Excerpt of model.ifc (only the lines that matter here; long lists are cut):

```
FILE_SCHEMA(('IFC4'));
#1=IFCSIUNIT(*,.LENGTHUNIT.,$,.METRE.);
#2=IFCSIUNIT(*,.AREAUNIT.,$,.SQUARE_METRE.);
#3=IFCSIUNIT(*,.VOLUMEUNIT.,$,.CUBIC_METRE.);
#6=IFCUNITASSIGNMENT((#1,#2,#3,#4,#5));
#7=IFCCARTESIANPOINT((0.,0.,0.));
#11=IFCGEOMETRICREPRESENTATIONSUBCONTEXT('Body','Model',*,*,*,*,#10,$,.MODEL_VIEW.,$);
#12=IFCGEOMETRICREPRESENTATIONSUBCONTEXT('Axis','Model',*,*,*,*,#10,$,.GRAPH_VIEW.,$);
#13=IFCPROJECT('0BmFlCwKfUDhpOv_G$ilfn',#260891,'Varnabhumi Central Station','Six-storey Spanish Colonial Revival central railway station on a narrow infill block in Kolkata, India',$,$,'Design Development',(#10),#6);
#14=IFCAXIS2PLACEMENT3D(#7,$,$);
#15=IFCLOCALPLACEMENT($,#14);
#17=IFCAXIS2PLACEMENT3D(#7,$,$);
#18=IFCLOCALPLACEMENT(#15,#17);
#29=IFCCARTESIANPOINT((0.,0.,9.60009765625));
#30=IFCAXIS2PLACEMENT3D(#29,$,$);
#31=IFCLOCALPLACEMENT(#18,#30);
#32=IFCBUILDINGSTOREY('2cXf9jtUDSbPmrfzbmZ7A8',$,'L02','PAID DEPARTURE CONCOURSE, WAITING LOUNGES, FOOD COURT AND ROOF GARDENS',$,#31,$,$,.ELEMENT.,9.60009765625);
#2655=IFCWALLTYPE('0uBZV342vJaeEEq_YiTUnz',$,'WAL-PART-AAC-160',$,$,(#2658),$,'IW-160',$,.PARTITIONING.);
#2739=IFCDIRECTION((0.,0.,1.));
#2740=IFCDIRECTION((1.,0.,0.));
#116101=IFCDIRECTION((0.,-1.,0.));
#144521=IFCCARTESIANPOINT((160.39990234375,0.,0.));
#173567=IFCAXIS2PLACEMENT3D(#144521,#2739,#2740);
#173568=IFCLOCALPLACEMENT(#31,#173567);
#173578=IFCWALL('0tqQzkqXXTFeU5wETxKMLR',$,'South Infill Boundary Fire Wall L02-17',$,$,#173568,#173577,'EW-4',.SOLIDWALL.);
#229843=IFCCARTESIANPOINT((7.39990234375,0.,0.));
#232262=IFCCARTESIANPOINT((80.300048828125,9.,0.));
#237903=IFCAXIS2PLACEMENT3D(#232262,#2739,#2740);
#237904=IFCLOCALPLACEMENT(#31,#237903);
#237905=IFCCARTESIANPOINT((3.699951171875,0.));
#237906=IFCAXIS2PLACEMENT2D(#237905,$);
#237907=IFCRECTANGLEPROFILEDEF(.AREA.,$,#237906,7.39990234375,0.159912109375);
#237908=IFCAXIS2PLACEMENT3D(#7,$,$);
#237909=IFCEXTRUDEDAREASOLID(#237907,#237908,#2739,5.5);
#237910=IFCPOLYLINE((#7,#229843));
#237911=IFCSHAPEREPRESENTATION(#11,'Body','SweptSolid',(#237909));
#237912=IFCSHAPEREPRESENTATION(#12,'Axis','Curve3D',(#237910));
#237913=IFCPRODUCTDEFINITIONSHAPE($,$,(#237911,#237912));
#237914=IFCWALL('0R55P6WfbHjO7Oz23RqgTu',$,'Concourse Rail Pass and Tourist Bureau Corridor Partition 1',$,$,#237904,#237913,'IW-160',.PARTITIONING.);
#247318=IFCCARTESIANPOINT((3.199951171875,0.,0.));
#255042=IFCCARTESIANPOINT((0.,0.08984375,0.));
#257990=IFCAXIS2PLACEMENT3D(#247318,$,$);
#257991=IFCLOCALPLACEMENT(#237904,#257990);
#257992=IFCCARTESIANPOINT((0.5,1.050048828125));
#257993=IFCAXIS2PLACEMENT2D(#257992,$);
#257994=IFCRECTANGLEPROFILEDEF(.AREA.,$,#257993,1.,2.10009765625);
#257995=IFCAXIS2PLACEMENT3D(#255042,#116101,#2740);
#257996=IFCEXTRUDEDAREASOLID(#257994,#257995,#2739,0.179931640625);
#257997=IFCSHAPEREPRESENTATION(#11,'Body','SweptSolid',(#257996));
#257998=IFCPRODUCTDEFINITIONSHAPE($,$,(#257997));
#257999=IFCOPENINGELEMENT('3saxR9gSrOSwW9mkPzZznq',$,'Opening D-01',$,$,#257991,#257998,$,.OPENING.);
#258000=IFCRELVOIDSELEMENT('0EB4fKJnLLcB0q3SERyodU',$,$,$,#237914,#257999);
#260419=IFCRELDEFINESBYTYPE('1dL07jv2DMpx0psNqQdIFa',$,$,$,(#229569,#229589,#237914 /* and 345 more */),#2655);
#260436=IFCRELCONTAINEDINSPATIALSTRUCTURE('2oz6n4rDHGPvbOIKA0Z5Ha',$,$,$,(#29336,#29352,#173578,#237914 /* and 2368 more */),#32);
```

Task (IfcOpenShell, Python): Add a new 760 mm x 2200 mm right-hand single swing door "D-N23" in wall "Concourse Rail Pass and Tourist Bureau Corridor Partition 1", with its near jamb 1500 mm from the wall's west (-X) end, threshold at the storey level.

```python
import numpy as np
import ifcopenshell
import ifcopenshell.api.feature
import ifcopenshell.api.geometry
import ifcopenshell.api.root
import ifcopenshell.api.spatial
import ifcopenshell.geom
import ifcopenshell.util.element
import ifcopenshell.util.placement
import ifcopenshell.util.representation
import ifcopenshell.util.shape
import ifcopenshell.util.unit

model = ifcopenshell.open("model.ifc")
unit_scale = ifcopenshell.util.unit.calculate_unit_scale(model)
settings = ifcopenshell.geom.settings()


def volume(element):
    """Net volume in cubic metres, openings subtracted."""
    shape = ifcopenshell.geom.create_shape(settings, element)
    return ifcopenshell.util.shape.get_volume(shape.geometry)


wall = model.by_guid("0R55P6WfbHjO7Oz23RqgTu")
storey = ifcopenshell.util.element.get_container(wall, ifc_class="IfcBuildingStorey")
context = ifcopenshell.util.representation.get_context(model, "Model", "Body", "MODEL_VIEW")
before = volume(wall)

width, height, from_end, sill = 0.76, 2.2, 1.5, 0.0  # metres

# The wall runs along its own X axis, and the end named is its -X end.
wall_shape = ifcopenshell.geom.create_shape(settings, wall)
x, y, z = ifcopenshell.util.shape.get_vertices(wall_shape.geometry).T
start = x.min() + from_end
face, thickness = float(y.min()), float(y.max() - y.min())
wall_matrix = ifcopenshell.util.placement.get_local_placement(wall.ObjectPlacement)
level = ifcopenshell.util.placement.get_local_placement(storey.ObjectPlacement)[2, 3]


def in_wall(x, y):
    """Placement at x, y metres in the wall's axes, at sill height."""
    matrix = wall_matrix.copy()
    matrix[:, 3] = wall_matrix @ np.array([x / unit_scale, y / unit_scale, 0.0, 1.0])
    matrix[2, 3] = level + sill / unit_scale
    return matrix


# Opening: a box that overshoots both wall faces by 50 mm.
opening = ifcopenshell.api.root.create_entity(model, ifc_class="IfcOpeningElement", predefined_type="OPENING")
box = ifcopenshell.api.geometry.add_wall_representation(
    model, context=context, length=width, height=height, thickness=thickness + 0.1
)
ifcopenshell.api.geometry.assign_representation(model, product=opening, representation=box)
ifcopenshell.api.geometry.edit_object_placement(model, product=opening, matrix=in_wall(start, face - 0.05), is_si=False)
ifcopenshell.api.feature.add_feature(model, feature=opening, element=wall)

door = ifcopenshell.api.root.create_entity(model, ifc_class="IfcDoor", name="D-N23", predefined_type="DOOR")
door.OverallWidth, door.OverallHeight = width / unit_scale, height / unit_scale
door.OperationType = "SINGLE_SWING_RIGHT"
body = ifcopenshell.api.geometry.add_door_representation(
    model,
    context=context,
    overall_width=door.OverallWidth,
    overall_height=door.OverallHeight,
    operation_type="SINGLE_SWING_RIGHT",
    lining_properties={"LiningDepth": thickness / unit_scale, "ThresholdDepth": thickness / unit_scale},
)
ifcopenshell.api.geometry.assign_representation(model, product=door, representation=body)
ifcopenshell.api.spatial.assign_container(model, products=[door], relating_structure=storey)
ifcopenshell.api.feature.add_filling(model, opening=opening, element=door)

# The lining spans the wall, so the door starts at the wall face.
ifcopenshell.api.geometry.edit_object_placement(model, product=door, matrix=in_wall(start, face), is_si=False)

after = volume(wall)

print(f"wall volume {before:.3f} -> {after:.3f} m3")

model.write("model_updated.ifc")
```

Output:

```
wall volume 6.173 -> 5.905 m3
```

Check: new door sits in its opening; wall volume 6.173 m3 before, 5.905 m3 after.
